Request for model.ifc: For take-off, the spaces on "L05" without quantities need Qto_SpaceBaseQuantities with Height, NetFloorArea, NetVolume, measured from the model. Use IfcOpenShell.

First a look at what the model holds.

```python
import ifcopenshell
import ifcopenshell.util.element
import ifcopenshell.util.unit

model = ifcopenshell.open("model.ifc")
print(model.schema)
for unit_type in ("LENGTHUNIT", "AREAUNIT", "VOLUMEUNIT"):
    print(unit_type, ifcopenshell.util.unit.calculate_unit_scale(model, unit_type))
storey = next(s for s in model.by_type("IfcBuildingStorey") if s.Name == "L05")
spaces = [e for e in ifcopenshell.util.element.get_decomposition(storey) if e.is_a("IfcSpace")]
for e in sorted(spaces, key=lambda e: e.id()):
    print(e.id(), e.is_a(), e.Name, list(ifcopenshell.util.element.get_psets(e, qtos_only=True)), sep=" | ")
```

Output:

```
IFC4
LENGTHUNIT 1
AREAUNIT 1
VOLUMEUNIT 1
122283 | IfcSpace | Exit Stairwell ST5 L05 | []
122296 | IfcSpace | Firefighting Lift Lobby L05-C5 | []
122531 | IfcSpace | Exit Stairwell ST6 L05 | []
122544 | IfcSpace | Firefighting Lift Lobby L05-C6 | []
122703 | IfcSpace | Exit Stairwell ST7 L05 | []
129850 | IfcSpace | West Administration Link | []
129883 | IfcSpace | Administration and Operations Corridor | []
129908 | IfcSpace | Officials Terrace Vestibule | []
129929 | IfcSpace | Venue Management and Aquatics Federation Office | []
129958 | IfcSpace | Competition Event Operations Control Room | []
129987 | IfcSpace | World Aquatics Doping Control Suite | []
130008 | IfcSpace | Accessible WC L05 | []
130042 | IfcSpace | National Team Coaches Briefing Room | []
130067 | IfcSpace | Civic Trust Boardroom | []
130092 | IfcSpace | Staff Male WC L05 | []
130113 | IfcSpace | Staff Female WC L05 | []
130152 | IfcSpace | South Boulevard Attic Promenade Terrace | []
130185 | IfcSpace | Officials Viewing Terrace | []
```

```python
import ifcopenshell
import ifcopenshell.api.pset
import ifcopenshell.geom
import ifcopenshell.util.element
import ifcopenshell.util.shape
import ifcopenshell.util.unit

model = ifcopenshell.open("model.ifc")
unit_scale = ifcopenshell.util.unit.calculate_unit_scale(model)
area_scale = ifcopenshell.util.unit.calculate_unit_scale(model, "AREAUNIT")
volume_scale = ifcopenshell.util.unit.calculate_unit_scale(model, "VOLUMEUNIT")
settings = ifcopenshell.geom.settings()

storey = next(s for s in model.by_type("IfcBuildingStorey") if s.Name == "L05")
spaces = [e for e in ifcopenshell.util.element.get_decomposition(storey) if e.is_a("IfcSpace")]

for e in sorted(spaces, key=lambda e: e.id()):
    if ifcopenshell.util.element.get_psets(e, qtos_only=True, should_inherit=False):
        continue
    # Geometry comes back in metres, in the element's own axes.
    shape = ifcopenshell.geom.create_shape(settings, e)
    values = {
        "Height": ifcopenshell.util.shape.get_z(shape.geometry) / unit_scale,
        "NetFloorArea": ifcopenshell.util.shape.get_footprint_area(shape.geometry) / area_scale,
        "NetVolume": ifcopenshell.util.shape.get_volume(shape.geometry) / volume_scale,
    }
    qto = ifcopenshell.api.pset.add_qto(model, product=e, name="Qto_SpaceBaseQuantities")
    ifcopenshell.api.pset.edit_qto(model, qto=qto, properties=values)
    print(e.id(), {k: round(v, 3) for k, v in values.items()})

model.write("model_edited.ifc")
```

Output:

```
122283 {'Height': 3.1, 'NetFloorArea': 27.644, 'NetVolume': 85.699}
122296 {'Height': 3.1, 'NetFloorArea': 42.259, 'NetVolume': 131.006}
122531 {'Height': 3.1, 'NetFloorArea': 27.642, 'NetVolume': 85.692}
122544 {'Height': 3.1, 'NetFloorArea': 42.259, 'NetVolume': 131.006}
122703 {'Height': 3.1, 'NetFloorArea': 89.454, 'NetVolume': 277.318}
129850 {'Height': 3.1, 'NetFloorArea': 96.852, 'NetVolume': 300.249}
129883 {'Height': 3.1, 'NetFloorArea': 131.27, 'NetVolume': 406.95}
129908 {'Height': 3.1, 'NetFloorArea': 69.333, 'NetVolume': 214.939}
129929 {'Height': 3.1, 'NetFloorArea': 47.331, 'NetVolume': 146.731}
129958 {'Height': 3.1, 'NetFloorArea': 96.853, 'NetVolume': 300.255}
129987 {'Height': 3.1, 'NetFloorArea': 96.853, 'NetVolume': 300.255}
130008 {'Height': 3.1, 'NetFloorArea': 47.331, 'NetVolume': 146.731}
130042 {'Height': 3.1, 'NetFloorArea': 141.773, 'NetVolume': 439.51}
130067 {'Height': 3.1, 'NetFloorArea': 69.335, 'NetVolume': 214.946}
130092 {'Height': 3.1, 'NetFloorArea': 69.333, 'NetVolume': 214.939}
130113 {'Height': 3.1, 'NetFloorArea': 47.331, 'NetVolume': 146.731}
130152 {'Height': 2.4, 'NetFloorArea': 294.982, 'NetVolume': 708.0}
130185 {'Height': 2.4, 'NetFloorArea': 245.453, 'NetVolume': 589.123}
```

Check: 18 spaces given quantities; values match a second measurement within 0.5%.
